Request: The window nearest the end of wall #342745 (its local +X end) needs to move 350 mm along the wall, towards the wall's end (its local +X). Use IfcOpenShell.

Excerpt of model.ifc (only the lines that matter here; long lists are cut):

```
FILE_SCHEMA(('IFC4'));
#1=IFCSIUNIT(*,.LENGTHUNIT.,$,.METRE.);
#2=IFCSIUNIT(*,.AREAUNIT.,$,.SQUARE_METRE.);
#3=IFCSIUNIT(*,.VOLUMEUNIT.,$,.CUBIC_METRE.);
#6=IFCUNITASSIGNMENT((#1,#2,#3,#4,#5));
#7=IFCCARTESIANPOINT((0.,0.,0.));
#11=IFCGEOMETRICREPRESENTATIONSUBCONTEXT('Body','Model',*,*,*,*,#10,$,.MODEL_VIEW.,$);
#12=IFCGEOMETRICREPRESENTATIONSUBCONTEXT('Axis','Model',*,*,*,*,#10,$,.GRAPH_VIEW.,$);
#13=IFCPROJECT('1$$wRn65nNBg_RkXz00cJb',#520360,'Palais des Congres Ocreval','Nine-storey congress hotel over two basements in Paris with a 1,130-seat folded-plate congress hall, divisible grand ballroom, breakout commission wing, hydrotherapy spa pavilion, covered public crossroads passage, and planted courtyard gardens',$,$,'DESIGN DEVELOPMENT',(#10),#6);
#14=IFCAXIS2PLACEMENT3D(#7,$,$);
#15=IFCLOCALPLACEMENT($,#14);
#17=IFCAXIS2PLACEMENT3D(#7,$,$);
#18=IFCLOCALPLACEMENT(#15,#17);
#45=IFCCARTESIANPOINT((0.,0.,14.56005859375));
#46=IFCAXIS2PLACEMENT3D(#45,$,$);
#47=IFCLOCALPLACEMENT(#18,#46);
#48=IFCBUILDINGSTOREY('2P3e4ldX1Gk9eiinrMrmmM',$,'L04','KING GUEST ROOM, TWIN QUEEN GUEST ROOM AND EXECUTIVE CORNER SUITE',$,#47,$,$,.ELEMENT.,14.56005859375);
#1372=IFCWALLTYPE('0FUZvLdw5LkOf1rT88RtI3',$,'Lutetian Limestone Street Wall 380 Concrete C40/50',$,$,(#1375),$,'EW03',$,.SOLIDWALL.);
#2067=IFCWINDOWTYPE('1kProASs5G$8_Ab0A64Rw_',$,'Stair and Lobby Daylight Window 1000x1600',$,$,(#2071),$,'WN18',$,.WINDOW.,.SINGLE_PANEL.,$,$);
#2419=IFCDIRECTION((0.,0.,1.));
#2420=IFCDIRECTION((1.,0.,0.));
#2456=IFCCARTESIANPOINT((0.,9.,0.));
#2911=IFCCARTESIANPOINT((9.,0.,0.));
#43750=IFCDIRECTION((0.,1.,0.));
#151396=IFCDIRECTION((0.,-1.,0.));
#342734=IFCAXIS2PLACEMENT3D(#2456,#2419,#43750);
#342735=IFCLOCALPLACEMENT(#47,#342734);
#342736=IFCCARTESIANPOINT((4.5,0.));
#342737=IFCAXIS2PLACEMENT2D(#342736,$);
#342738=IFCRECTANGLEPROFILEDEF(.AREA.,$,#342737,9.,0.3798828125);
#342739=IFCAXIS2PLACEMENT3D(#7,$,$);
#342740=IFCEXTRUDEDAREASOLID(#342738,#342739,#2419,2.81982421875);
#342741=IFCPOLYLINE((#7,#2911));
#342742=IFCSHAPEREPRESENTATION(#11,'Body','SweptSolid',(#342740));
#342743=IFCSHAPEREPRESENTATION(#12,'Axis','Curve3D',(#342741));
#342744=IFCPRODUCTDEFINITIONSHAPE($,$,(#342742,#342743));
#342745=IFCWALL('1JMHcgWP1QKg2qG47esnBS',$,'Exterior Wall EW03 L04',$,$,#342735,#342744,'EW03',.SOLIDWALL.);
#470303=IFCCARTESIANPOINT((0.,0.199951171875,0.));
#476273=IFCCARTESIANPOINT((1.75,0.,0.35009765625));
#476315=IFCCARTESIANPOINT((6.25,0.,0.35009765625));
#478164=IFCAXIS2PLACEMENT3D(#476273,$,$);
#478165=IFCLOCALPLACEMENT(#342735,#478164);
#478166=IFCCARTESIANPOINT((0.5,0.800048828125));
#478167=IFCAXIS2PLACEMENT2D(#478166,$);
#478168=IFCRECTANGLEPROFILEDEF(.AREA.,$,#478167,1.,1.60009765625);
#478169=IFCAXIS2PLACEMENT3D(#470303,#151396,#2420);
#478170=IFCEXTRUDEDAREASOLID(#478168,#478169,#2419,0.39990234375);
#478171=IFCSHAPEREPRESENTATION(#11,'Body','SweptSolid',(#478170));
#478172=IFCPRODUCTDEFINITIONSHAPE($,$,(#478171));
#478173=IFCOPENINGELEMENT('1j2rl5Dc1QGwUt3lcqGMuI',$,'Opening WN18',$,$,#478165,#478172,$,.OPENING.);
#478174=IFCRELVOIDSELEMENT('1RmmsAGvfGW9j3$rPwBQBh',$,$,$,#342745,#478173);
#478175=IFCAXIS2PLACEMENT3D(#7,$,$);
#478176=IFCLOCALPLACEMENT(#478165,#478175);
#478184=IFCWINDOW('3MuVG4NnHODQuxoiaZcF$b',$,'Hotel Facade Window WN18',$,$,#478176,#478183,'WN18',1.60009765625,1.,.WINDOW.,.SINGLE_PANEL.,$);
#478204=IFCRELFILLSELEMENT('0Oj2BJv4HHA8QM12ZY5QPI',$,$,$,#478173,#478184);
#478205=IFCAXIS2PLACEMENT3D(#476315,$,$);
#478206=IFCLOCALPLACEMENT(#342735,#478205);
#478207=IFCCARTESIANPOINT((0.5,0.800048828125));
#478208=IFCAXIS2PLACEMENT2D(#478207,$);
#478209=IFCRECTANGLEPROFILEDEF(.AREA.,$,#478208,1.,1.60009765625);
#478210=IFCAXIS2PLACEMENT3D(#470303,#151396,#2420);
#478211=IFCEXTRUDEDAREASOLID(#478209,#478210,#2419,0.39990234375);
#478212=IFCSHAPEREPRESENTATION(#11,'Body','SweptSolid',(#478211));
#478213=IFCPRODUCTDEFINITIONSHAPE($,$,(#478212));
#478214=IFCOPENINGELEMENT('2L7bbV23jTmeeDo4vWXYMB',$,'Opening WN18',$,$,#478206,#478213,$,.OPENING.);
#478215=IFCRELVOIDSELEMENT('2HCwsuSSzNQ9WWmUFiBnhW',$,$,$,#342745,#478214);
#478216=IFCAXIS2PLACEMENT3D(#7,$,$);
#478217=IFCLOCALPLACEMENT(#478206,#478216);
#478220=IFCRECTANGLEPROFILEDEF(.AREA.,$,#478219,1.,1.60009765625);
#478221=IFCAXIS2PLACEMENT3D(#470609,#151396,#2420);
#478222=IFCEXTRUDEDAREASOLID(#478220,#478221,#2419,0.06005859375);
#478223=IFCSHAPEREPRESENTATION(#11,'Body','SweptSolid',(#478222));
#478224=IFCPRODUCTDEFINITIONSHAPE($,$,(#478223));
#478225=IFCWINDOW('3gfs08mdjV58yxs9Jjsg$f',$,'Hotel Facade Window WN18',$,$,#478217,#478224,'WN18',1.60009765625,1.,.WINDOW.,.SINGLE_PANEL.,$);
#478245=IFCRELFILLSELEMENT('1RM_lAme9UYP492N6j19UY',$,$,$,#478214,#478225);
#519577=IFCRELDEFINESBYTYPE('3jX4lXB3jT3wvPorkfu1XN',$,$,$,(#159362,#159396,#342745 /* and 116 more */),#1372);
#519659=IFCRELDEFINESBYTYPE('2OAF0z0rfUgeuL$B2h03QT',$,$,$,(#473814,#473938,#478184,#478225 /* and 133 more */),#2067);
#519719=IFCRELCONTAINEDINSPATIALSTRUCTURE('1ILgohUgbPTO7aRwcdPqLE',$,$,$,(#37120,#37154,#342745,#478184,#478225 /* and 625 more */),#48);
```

```python
import ifcopenshell
import ifcopenshell.api.geometry
import ifcopenshell.util.placement
import ifcopenshell.util.unit

model = ifcopenshell.open("model.ifc")
unit_scale = ifcopenshell.util.unit.calculate_unit_scale(model)

window = model.by_guid("3gfs08mdjV58yxs9Jjsg$f")
opening = window.FillsVoids[0].RelatingOpeningElement
wall = opening.VoidsElements[0].RelatingBuildingElement

wall_matrix = ifcopenshell.util.placement.get_local_placement(wall.ObjectPlacement)
shift = wall_matrix[:3, 0] * 0.35 / unit_scale
before = ifcopenshell.util.placement.get_local_placement(window.ObjectPlacement)[:3, 3].copy()

# The window is placed relative to its opening, so it follows when the opening moves.
matrix = ifcopenshell.util.placement.get_local_placement(opening.ObjectPlacement)
matrix[:3, 3] += shift
ifcopenshell.api.geometry.edit_object_placement(
    model, product=opening, matrix=matrix, is_si=False, should_transform_children=True
)

after = ifcopenshell.util.placement.get_local_placement(window.ObjectPlacement)[:3, 3]
print("window moved by", (after - before).round(3) + 0.0)

model.write("model_edited.ifc")
```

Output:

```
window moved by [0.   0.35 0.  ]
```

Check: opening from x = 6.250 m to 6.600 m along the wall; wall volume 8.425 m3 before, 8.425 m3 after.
